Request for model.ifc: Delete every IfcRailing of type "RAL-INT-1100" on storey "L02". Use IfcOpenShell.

First a look at what the model holds.

```python
import ifcopenshell
import ifcopenshell.util.element

model = ifcopenshell.open("model.ifc")
print(model.schema)
storey = next(s for s in model.by_type("IfcBuildingStorey") if s.Name == "L02")
railings = [e for e in ifcopenshell.util.element.get_decomposition(storey) if e.is_a("IfcRailing")]
seen = {}
for e in railings:
    element_type = ifcopenshell.util.element.get_type(e)
    name = element_type.Name if element_type not in (None, e) else None
    seen[name] = seen.get(name, 0) + 1
for name, count in sorted(seen.items(), key=str):
    print(count, "x", name)
```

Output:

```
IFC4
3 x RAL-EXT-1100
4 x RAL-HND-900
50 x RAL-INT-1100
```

```python
import ifcopenshell
import ifcopenshell.api.root
import ifcopenshell.util.element

model = ifcopenshell.open("model.ifc")

storey = next(s for s in model.by_type("IfcBuildingStorey") if s.Name == "L02")
railings = [e for e in ifcopenshell.util.element.get_decomposition(storey) if e.is_a("IfcRailing")]
targets = [e for e in railings if (t := ifcopenshell.util.element.get_type(e)) not in (None, e) and t.Name == "RAL-INT-1100"]

for e in targets:
    ifcopenshell.api.root.remove_product(model, product=e)
print(len(targets), "removed")

model.write("model_edited.ifc")
```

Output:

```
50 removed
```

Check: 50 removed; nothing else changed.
